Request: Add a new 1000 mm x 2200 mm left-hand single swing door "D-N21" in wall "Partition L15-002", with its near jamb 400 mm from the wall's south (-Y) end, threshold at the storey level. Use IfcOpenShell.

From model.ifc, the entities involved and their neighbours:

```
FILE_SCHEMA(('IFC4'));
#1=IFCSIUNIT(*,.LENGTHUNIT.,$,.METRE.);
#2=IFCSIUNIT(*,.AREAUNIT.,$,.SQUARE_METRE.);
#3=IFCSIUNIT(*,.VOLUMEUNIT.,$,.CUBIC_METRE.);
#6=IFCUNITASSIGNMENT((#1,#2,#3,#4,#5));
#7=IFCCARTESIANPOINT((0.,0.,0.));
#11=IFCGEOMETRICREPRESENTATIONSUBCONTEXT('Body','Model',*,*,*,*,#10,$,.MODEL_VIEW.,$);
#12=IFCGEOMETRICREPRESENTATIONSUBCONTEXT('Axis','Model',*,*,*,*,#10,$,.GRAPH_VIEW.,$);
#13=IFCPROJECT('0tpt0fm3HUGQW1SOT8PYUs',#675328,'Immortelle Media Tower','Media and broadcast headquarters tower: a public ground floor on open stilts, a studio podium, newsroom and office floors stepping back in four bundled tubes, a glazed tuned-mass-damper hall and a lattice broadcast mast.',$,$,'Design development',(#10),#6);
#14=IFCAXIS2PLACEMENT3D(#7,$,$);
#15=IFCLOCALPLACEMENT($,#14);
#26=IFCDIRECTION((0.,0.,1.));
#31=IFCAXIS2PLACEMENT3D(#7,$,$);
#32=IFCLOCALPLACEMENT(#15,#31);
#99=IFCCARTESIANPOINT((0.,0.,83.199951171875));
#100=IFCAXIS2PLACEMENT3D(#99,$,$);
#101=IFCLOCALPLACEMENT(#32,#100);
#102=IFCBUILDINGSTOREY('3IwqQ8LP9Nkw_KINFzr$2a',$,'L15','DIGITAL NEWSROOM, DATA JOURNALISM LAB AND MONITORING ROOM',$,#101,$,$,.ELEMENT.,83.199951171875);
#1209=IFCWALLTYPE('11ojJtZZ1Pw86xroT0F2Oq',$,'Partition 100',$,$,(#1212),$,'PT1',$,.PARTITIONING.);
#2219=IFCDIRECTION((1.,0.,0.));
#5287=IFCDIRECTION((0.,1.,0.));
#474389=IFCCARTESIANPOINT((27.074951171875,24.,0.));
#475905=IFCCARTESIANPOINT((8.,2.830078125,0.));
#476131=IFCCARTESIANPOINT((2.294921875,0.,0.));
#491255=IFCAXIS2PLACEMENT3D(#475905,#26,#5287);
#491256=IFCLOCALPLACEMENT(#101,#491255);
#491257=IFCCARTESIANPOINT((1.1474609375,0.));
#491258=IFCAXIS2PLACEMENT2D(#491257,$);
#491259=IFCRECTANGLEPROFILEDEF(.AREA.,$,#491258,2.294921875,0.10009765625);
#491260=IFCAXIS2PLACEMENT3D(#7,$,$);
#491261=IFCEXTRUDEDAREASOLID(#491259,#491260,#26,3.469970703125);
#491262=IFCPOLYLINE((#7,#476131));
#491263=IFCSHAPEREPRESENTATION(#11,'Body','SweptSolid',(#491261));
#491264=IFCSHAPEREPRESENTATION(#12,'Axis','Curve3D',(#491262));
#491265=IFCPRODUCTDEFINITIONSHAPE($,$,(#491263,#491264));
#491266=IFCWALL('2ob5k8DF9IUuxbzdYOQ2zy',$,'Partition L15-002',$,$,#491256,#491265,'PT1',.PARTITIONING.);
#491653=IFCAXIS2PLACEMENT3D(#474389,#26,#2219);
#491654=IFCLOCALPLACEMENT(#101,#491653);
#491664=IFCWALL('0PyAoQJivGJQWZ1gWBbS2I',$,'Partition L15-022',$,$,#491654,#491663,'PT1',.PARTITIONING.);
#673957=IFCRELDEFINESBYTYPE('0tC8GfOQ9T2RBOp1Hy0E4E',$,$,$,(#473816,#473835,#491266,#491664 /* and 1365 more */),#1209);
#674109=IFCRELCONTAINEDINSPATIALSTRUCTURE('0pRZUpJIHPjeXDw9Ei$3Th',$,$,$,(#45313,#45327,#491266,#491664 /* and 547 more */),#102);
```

```python
import numpy as np
import ifcopenshell
import ifcopenshell.api.feature
import ifcopenshell.api.geometry
import ifcopenshell.api.root
import ifcopenshell.api.spatial
import ifcopenshell.geom
import ifcopenshell.util.element
import ifcopenshell.util.placement
import ifcopenshell.util.representation
import ifcopenshell.util.shape
import ifcopenshell.util.unit

model = ifcopenshell.open("model.ifc")
unit_scale = ifcopenshell.util.unit.calculate_unit_scale(model)
settings = ifcopenshell.geom.settings()


def volume(element):
    """Net volume in cubic metres, openings subtracted."""
    shape = ifcopenshell.geom.create_shape(settings, element)
    return ifcopenshell.util.shape.get_volume(shape.geometry)


wall = model.by_id(491266)
storey = ifcopenshell.util.element.get_container(wall, ifc_class="IfcBuildingStorey")
context = ifcopenshell.util.representation.get_context(model, "Model", "Body", "MODEL_VIEW")
before = volume(wall)

width, height, from_end, sill = 1, 2.2, 0.4, 0.0  # metres

# The wall runs along its own X axis, and the end named is its -X end.
wall_shape = ifcopenshell.geom.create_shape(settings, wall)
x, y, z = ifcopenshell.util.shape.get_vertices(wall_shape.geometry).T
start = x.min() + from_end
face, thickness = float(y.min()), float(y.max() - y.min())
wall_matrix = ifcopenshell.util.placement.get_local_placement(wall.ObjectPlacement)
level = ifcopenshell.util.placement.get_local_placement(storey.ObjectPlacement)[2, 3]


def in_wall(x, y):
    """Placement at x, y metres in the wall's axes, at sill height."""
    matrix = wall_matrix.copy()
    matrix[:, 3] = wall_matrix @ np.array([x / unit_scale, y / unit_scale, 0.0, 1.0])
    matrix[2, 3] = level + sill / unit_scale
    return matrix


# Opening: a box that overshoots both wall faces by 50 mm.
opening = ifcopenshell.api.root.create_entity(model, ifc_class="IfcOpeningElement", predefined_type="OPENING")
box = ifcopenshell.api.geometry.add_wall_representation(
    model, context=context, length=width, height=height, thickness=thickness + 0.1
)
ifcopenshell.api.geometry.assign_representation(model, product=opening, representation=box)
ifcopenshell.api.geometry.edit_object_placement(model, product=opening, matrix=in_wall(start, face - 0.05), is_si=False)
ifcopenshell.api.feature.add_feature(model, feature=opening, element=wall)

door = ifcopenshell.api.root.create_entity(model, ifc_class="IfcDoor", name="D-N21", predefined_type="DOOR")
door.OverallWidth, door.OverallHeight = width / unit_scale, height / unit_scale
door.OperationType = "SINGLE_SWING_LEFT"
body = ifcopenshell.api.geometry.add_door_representation(
    model,
    context=context,
    overall_width=door.OverallWidth,
    overall_height=door.OverallHeight,
    operation_type="SINGLE_SWING_LEFT",
    lining_properties={"LiningDepth": thickness / unit_scale, "ThresholdDepth": thickness / unit_scale},
)
ifcopenshell.api.geometry.assign_representation(model, product=door, representation=body)
ifcopenshell.api.spatial.assign_container(model, products=[door], relating_structure=storey)
ifcopenshell.api.feature.add_filling(model, opening=opening, element=door)

# The lining spans the wall, so the door starts at the wall face.
ifcopenshell.api.geometry.edit_object_placement(model, product=door, matrix=in_wall(start, face), is_si=False)

after = volume(wall)

print(f"wall volume {before:.3f} -> {after:.3f} m3")

model.write("model_edited.ifc")
```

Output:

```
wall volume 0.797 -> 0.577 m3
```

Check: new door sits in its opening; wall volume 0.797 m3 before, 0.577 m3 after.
